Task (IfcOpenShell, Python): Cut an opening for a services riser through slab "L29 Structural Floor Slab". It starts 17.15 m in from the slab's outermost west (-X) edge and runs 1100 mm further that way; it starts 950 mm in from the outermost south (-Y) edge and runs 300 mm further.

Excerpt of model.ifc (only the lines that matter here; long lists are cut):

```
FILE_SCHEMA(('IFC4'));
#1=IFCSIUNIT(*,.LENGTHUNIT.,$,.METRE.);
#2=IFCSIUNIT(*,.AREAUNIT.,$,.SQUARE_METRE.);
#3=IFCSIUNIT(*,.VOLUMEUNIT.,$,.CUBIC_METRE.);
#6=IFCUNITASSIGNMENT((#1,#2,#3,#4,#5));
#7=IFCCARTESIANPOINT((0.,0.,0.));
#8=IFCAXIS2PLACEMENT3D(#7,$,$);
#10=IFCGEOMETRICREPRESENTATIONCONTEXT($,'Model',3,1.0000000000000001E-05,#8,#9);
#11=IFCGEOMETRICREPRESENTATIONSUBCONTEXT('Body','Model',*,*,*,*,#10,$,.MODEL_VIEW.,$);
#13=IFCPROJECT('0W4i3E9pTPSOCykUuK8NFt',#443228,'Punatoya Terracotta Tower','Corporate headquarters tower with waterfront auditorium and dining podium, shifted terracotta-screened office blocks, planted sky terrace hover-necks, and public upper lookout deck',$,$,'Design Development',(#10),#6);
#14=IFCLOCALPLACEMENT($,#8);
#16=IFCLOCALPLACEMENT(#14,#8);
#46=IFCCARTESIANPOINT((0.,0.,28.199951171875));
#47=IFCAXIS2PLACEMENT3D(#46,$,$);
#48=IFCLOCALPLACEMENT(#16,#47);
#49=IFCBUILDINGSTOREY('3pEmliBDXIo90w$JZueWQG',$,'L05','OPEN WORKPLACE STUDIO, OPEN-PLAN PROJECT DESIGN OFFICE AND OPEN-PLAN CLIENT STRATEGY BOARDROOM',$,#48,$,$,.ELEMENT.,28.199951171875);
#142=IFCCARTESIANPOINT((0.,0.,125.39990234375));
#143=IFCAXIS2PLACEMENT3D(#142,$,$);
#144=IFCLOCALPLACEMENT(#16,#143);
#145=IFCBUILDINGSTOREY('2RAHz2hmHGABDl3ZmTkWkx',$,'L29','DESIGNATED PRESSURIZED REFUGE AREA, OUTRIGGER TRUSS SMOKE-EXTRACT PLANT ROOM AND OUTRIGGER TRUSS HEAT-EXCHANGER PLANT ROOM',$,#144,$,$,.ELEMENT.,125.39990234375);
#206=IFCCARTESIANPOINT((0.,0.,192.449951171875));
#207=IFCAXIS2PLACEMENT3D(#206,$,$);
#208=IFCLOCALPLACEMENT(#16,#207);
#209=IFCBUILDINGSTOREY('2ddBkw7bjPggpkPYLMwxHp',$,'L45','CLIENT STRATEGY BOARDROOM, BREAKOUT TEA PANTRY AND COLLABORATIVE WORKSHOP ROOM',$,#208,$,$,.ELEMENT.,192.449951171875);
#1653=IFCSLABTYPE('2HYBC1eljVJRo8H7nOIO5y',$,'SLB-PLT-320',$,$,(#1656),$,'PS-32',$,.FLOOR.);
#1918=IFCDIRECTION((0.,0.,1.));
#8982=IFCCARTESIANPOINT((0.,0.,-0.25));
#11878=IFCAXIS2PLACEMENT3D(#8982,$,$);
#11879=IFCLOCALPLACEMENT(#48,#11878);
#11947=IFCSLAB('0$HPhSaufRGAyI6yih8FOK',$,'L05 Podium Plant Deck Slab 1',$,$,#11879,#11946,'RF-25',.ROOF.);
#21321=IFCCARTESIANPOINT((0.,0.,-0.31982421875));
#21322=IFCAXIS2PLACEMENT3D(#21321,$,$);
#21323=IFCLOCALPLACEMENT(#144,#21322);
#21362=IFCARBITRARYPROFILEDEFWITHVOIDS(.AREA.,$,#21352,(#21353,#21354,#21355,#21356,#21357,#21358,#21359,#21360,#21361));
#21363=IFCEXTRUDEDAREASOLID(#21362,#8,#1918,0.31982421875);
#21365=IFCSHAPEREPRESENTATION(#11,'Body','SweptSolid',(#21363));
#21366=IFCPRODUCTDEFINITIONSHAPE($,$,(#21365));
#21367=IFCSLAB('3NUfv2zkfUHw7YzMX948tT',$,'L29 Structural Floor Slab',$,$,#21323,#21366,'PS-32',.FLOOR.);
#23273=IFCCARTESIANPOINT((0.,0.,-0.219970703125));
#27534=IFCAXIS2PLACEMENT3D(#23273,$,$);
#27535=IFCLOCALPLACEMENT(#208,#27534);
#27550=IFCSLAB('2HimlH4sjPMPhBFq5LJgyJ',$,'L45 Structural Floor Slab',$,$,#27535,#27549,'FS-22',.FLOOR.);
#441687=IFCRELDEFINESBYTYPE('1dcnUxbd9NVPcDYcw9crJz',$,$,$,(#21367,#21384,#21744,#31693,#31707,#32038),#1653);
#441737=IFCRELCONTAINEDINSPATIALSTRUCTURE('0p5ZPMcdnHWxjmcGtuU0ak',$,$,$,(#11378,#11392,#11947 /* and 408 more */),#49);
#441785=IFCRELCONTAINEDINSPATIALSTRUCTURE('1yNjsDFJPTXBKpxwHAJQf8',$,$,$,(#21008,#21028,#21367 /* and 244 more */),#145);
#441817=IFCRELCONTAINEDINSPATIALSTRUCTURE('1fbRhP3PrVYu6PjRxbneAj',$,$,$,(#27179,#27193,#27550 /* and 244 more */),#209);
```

```python
import numpy as np
import ifcopenshell
import ifcopenshell.api.feature
import ifcopenshell.api.geometry
import ifcopenshell.api.root
import ifcopenshell.geom
import ifcopenshell.util.placement
import ifcopenshell.util.representation
import ifcopenshell.util.shape
import ifcopenshell.util.unit

model = ifcopenshell.open("model.ifc")
unit_scale = ifcopenshell.util.unit.calculate_unit_scale(model)
settings = ifcopenshell.geom.settings()


def volume(element):
    """Net volume in cubic metres, openings subtracted."""
    shape = ifcopenshell.geom.create_shape(settings, element)
    return ifcopenshell.util.shape.get_volume(shape.geometry)


slab = model.by_guid("3NUfv2zkfUHw7YzMX948tT")
before = volume(slab)

# Extent in the slab's own axes, in metres. The edges named are its -X and -Y sides.
slab_shape = ifcopenshell.geom.create_shape(settings, slab)
vertices = ifcopenshell.util.shape.get_vertices(slab_shape.geometry)
x_min, y_min, bottom = vertices.min(axis=0)
top = vertices[:, 2].max()

opening = ifcopenshell.api.root.create_entity(model, ifc_class="IfcOpeningElement", name="Services riser opening", predefined_type="OPENING")
context = ifcopenshell.util.representation.get_context(model, "Model", "Body", "MODEL_VIEW")
width, depth = 1.1, 0.3
outline = [(0.0, 0.0), (width, 0.0), (width, depth), (0.0, depth), (0.0, 0.0)]
# Overshoot both faces by 50 mm so the cut is clean.
shape = ifcopenshell.api.geometry.add_slab_representation(
    model, context=context, depth=top - bottom + 0.1, polyline=outline
)
ifcopenshell.api.geometry.assign_representation(model, product=opening, representation=shape)

matrix = ifcopenshell.util.placement.get_local_placement(slab.ObjectPlacement)
matrix[:, 3] = matrix @ np.append(np.array([x_min + 17.15, y_min + 0.95, bottom - 0.05]) / unit_scale, 1.0)
ifcopenshell.api.geometry.edit_object_placement(model, product=opening, matrix=matrix, is_si=False)
ifcopenshell.api.feature.add_feature(model, feature=opening, element=slab)

after = volume(slab)

print(f"slab volume {before:.3f} -> {after:.3f} m3")

model.write("model_v2.ifc")
```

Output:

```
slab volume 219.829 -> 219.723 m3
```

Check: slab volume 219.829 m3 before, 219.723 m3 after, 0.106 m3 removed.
